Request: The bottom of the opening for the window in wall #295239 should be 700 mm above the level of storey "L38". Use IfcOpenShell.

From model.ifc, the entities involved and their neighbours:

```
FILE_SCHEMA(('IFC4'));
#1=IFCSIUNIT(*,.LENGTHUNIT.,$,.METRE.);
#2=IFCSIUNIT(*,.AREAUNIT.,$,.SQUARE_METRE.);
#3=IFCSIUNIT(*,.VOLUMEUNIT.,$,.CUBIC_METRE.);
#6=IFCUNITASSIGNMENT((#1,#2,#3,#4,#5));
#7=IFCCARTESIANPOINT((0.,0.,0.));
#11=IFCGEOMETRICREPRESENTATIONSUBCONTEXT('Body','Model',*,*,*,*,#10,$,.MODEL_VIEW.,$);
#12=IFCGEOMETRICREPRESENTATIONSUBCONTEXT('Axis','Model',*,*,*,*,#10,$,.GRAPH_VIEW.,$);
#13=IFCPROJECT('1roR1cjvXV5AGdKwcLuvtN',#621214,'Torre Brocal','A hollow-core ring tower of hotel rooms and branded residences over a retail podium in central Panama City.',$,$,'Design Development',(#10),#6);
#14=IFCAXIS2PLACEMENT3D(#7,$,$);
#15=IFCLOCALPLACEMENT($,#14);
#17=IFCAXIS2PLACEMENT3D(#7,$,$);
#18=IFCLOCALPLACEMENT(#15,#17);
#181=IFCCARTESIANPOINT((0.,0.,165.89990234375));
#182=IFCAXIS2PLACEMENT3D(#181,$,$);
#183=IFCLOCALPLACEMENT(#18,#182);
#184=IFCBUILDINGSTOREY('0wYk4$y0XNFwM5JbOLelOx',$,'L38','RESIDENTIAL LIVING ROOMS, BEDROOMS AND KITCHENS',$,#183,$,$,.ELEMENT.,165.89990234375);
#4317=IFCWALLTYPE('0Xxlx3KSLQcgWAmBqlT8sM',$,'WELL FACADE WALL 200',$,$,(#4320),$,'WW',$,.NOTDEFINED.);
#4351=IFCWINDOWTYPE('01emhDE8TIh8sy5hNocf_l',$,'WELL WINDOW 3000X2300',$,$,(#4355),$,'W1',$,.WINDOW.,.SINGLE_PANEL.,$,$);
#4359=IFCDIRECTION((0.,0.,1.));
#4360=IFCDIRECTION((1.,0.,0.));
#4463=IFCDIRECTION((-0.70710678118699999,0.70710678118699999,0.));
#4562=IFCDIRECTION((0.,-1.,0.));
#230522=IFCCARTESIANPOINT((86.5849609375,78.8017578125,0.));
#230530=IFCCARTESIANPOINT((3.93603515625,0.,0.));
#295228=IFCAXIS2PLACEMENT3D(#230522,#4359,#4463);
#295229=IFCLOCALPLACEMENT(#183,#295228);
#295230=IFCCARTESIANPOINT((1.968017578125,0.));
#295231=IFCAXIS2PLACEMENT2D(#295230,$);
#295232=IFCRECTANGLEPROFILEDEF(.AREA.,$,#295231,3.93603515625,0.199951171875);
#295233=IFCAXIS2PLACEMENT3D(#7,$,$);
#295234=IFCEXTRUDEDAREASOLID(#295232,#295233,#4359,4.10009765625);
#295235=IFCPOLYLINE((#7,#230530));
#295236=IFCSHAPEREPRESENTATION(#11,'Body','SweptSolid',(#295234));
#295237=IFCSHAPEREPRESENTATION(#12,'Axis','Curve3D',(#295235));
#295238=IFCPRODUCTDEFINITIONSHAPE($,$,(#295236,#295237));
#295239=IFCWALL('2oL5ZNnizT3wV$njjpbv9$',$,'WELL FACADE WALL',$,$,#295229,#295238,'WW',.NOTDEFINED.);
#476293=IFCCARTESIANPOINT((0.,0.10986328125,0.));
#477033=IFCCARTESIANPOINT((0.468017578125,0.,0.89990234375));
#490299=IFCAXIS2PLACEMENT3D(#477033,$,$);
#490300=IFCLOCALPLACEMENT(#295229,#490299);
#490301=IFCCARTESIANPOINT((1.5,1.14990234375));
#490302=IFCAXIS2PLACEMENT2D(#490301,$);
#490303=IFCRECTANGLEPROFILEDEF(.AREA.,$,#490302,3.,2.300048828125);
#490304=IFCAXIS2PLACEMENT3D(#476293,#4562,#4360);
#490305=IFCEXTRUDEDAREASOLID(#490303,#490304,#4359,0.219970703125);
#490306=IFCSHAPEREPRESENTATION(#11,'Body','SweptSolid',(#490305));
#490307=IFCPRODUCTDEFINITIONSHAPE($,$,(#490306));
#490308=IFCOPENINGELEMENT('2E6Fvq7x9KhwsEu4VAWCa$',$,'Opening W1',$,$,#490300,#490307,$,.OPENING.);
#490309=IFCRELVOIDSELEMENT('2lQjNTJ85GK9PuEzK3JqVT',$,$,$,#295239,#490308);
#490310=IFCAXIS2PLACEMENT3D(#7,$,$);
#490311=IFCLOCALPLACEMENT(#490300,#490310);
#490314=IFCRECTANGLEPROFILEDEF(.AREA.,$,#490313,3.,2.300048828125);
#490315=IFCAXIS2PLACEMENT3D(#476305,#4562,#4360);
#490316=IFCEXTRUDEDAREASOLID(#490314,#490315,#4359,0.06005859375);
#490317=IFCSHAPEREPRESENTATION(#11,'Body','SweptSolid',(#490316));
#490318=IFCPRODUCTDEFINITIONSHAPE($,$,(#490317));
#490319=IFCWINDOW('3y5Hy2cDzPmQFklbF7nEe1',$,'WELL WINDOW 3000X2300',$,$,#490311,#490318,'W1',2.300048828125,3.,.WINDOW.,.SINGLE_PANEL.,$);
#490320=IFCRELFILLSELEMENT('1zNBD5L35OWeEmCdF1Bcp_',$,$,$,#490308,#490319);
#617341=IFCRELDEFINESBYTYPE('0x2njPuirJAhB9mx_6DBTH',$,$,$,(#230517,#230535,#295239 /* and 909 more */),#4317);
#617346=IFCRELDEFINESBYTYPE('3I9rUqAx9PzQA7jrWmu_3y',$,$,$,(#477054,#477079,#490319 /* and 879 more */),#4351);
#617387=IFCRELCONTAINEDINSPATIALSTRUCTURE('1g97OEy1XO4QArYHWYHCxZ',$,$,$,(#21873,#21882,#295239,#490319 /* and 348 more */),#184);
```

```python
import numpy as np
import ifcopenshell
import ifcopenshell.api.geometry
import ifcopenshell.geom
import ifcopenshell.util.element
import ifcopenshell.util.placement
import ifcopenshell.util.shape
import ifcopenshell.util.unit

model = ifcopenshell.open("model.ifc")
unit_scale = ifcopenshell.util.unit.calculate_unit_scale(model)

window = model.by_id(490319)
opening = window.FillsVoids[0].RelatingOpeningElement
storey = ifcopenshell.util.element.get_container(window, ifc_class="IfcBuildingStorey")
level = ifcopenshell.util.placement.get_local_placement(storey.ObjectPlacement)[2, 3]

# The opening's origin need not be at the sill, so measure its lowest point.
shape = ifcopenshell.geom.create_shape(ifcopenshell.geom.settings(), opening)
bottom = ifcopenshell.util.shape.get_shape_bottom_elevation(shape, shape.geometry) / unit_scale
dz = level + 0.7 / unit_scale - bottom

shift = np.array([0.0, 0.0, dz])
# The window is placed relative to its opening, so it follows when the opening moves.
matrix = ifcopenshell.util.placement.get_local_placement(opening.ObjectPlacement)
matrix[:3, 3] += shift
ifcopenshell.api.geometry.edit_object_placement(
    model, product=opening, matrix=matrix, is_si=False, should_transform_children=True
)

print(f"moved by {dz * unit_scale:+.3f} m")

model.write("model_updated.ifc")
```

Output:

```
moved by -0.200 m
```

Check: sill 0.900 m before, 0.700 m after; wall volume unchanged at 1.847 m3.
